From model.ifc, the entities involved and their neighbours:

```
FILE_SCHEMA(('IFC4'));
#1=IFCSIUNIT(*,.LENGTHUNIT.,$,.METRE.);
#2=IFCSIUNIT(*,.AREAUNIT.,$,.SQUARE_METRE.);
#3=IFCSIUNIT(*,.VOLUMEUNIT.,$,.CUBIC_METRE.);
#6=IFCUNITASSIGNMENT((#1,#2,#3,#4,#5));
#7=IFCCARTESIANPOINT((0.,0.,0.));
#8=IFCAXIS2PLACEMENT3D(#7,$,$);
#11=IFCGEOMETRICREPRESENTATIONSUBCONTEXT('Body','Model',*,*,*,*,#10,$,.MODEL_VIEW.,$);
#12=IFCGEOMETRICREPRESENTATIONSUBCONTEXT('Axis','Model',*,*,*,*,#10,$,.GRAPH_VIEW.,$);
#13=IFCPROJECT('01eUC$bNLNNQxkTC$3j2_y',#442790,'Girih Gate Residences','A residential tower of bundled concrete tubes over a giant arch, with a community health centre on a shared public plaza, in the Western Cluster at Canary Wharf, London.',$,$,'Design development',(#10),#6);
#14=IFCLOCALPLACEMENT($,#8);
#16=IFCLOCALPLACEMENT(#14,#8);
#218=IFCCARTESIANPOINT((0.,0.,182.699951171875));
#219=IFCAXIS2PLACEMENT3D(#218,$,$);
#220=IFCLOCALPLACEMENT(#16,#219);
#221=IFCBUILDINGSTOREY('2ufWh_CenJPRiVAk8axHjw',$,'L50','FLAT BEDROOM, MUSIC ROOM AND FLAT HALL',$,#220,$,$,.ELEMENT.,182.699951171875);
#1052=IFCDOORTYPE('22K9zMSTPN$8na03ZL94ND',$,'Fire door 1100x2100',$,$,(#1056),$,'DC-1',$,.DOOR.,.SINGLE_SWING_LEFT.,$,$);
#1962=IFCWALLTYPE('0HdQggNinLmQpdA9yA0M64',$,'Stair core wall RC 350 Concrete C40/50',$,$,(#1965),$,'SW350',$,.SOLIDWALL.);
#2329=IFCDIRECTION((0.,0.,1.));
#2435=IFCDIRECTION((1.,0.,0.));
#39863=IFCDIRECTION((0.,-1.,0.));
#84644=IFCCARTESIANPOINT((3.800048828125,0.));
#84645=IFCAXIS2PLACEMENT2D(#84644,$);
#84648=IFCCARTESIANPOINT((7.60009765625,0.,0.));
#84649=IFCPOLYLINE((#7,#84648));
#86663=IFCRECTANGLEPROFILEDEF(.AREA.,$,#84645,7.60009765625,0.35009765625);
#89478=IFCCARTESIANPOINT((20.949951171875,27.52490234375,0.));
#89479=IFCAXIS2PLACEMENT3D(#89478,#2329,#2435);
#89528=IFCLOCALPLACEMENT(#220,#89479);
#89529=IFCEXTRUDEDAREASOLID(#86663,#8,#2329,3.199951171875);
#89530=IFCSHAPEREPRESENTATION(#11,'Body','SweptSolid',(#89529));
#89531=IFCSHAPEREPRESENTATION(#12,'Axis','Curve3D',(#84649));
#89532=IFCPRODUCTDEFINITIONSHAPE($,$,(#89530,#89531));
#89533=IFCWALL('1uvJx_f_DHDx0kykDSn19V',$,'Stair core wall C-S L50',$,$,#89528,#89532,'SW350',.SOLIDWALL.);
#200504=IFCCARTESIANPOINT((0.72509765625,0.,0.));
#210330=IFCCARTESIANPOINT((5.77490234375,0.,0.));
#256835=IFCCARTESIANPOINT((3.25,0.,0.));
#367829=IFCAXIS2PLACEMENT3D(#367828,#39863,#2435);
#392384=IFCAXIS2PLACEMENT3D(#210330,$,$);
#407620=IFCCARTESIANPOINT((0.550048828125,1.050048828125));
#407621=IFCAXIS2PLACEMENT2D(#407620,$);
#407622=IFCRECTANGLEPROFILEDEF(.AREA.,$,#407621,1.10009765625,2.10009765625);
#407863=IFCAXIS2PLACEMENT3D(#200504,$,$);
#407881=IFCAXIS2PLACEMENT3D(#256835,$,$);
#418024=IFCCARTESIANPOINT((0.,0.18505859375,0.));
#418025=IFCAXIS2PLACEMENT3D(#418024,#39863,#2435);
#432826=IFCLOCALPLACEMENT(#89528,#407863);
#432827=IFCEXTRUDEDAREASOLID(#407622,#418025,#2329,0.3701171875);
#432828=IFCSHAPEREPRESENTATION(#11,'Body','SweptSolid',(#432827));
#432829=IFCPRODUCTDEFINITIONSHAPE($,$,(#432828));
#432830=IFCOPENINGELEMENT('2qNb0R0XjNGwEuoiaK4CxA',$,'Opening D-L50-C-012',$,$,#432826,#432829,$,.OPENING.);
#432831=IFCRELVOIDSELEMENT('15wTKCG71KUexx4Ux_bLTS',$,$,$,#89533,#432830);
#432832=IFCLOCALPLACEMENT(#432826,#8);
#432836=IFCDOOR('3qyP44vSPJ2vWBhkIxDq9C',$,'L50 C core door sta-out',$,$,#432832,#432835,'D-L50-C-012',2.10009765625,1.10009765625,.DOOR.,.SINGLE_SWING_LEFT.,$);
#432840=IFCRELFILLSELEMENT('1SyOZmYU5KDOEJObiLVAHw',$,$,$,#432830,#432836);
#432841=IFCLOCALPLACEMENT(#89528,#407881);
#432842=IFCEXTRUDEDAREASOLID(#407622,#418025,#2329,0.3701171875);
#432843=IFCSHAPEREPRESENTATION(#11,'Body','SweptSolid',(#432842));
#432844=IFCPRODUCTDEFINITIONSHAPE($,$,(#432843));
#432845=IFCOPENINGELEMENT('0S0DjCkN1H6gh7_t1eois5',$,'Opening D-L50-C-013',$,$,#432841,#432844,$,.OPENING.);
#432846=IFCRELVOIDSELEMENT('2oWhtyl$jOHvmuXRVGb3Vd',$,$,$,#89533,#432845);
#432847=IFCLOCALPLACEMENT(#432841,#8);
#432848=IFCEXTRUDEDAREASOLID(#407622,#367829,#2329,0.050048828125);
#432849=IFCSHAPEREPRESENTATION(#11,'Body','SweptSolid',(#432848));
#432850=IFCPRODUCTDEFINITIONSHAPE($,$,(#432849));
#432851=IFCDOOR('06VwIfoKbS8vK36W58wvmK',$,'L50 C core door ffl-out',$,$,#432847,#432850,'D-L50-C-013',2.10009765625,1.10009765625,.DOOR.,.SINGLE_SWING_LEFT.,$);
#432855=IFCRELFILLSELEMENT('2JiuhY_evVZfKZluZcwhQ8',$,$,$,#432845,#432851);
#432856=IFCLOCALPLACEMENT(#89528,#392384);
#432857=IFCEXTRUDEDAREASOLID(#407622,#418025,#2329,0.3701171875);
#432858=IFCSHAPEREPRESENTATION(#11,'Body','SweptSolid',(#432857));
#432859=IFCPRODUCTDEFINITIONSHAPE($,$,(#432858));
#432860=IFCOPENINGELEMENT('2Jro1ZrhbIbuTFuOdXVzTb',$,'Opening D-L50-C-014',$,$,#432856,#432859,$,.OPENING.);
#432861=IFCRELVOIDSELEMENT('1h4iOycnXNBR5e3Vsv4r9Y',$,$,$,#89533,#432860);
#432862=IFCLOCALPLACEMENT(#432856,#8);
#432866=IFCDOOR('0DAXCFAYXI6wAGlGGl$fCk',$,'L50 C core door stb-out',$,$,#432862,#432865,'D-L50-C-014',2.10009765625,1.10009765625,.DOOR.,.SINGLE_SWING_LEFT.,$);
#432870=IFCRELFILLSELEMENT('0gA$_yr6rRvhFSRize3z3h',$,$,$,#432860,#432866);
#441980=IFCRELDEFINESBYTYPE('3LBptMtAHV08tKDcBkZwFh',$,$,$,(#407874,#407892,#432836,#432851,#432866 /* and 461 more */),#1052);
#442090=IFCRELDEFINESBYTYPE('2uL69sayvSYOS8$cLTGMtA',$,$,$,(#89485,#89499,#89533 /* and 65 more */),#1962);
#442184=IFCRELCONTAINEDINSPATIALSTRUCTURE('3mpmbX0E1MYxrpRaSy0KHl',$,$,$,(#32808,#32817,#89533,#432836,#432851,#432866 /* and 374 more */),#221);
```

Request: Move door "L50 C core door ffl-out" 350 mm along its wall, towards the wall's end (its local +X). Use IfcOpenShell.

```python
import ifcopenshell
import ifcopenshell.api.geometry
import ifcopenshell.util.placement
import ifcopenshell.util.unit

model = ifcopenshell.open("model.ifc")
unit_scale = ifcopenshell.util.unit.calculate_unit_scale(model)

door = model.by_guid("06VwIfoKbS8vK36W58wvmK")
opening = door.FillsVoids[0].RelatingOpeningElement
wall = opening.VoidsElements[0].RelatingBuildingElement

wall_matrix = ifcopenshell.util.placement.get_local_placement(wall.ObjectPlacement)
shift = wall_matrix[:3, 0] * 0.35 / unit_scale
before = ifcopenshell.util.placement.get_local_placement(door.ObjectPlacement)[:3, 3].copy()

# The door is placed relative to its opening, so it follows when the opening moves.
matrix = ifcopenshell.util.placement.get_local_placement(opening.ObjectPlacement)
matrix[:3, 3] += shift
ifcopenshell.api.geometry.edit_object_placement(
    model, product=opening, matrix=matrix, is_si=False, should_transform_children=True
)

after = ifcopenshell.util.placement.get_local_placement(door.ObjectPlacement)[:3, 3]
print("door moved by", (after - before).round(3) + 0.0)

model.write("model_edited.ifc")
```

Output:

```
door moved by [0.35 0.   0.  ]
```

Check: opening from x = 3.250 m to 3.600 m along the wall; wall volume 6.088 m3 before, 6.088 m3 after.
